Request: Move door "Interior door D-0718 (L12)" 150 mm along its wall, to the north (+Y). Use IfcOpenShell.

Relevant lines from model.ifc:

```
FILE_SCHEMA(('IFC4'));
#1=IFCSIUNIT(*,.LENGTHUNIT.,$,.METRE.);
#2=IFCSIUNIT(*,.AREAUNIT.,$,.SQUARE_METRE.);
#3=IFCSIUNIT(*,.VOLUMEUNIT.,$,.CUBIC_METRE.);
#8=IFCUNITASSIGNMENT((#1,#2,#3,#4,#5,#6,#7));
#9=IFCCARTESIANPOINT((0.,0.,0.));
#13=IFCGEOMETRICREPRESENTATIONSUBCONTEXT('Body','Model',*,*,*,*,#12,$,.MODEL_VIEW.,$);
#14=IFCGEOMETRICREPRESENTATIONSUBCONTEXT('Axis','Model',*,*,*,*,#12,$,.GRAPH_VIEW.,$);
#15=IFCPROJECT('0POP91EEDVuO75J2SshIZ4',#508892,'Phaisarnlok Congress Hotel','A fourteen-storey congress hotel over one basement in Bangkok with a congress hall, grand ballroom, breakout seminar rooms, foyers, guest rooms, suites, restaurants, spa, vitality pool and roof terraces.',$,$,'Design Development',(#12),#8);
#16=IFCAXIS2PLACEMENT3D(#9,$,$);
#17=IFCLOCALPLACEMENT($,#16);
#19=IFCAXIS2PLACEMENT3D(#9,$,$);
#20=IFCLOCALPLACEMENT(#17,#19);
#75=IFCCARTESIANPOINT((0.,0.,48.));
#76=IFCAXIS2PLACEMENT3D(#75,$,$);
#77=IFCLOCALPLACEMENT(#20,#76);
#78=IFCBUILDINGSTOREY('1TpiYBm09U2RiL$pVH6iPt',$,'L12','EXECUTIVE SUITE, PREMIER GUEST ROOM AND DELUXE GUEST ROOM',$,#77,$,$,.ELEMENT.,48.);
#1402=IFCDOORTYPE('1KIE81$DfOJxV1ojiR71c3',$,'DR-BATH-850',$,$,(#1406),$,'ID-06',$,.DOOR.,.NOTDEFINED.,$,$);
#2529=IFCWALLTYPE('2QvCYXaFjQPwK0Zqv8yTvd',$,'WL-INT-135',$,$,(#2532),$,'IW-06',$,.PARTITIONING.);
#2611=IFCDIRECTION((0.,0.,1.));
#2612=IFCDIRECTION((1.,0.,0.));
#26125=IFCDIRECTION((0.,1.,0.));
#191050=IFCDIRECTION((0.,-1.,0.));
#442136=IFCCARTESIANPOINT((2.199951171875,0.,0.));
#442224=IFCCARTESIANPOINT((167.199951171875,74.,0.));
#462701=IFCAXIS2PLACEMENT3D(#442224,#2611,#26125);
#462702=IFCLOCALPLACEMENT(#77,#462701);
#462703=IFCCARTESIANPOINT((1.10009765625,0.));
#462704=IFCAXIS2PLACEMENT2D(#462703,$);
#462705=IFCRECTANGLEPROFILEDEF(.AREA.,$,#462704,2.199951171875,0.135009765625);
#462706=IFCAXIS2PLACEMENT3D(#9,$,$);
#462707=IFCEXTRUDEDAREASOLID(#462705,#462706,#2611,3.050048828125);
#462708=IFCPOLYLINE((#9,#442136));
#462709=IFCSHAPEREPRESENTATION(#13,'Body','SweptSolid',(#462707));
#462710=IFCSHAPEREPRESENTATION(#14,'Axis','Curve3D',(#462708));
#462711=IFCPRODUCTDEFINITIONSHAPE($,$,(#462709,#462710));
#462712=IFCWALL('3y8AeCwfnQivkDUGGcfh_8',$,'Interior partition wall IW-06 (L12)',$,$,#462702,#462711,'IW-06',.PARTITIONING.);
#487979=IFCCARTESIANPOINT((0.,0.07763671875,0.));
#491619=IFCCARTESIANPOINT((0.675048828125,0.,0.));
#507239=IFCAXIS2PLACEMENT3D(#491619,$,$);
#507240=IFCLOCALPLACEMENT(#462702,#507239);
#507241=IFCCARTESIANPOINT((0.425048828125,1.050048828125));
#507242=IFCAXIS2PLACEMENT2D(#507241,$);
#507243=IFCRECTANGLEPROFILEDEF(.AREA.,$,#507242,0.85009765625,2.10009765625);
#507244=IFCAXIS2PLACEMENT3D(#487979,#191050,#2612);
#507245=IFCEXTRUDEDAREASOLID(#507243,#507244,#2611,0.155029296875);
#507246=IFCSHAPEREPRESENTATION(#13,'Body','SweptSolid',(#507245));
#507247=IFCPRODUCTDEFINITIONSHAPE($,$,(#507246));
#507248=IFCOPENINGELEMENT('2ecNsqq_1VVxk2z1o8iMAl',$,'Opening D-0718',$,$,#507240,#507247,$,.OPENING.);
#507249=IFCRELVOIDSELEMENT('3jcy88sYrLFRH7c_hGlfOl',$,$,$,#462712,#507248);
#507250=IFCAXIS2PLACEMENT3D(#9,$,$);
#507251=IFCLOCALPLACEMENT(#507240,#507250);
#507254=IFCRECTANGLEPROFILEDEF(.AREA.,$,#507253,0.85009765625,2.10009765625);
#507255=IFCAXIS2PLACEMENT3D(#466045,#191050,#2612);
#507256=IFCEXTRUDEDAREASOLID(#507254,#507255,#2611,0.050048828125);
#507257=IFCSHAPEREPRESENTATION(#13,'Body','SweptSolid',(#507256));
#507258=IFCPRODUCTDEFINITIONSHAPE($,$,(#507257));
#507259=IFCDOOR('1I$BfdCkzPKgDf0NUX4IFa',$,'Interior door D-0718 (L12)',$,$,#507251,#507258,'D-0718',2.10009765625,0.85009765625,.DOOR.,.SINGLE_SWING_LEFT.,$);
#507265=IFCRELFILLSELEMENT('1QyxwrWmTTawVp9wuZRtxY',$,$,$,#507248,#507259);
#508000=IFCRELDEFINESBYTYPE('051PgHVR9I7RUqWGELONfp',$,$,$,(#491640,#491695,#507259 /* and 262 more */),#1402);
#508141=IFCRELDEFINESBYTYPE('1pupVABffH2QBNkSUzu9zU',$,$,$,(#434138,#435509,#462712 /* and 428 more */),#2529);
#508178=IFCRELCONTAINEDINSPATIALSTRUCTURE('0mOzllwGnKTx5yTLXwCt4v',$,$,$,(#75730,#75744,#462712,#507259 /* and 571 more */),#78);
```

```python
import ifcopenshell
import ifcopenshell.api.geometry
import ifcopenshell.util.placement
import ifcopenshell.util.unit

model = ifcopenshell.open("model.ifc")
unit_scale = ifcopenshell.util.unit.calculate_unit_scale(model)

door = model.by_guid("1I$BfdCkzPKgDf0NUX4IFa")
opening = door.FillsVoids[0].RelatingOpeningElement
wall = opening.VoidsElements[0].RelatingBuildingElement

wall_matrix = ifcopenshell.util.placement.get_local_placement(wall.ObjectPlacement)
shift = wall_matrix[:3, 0] * 0.15 / unit_scale
before = ifcopenshell.util.placement.get_local_placement(door.ObjectPlacement)[:3, 3].copy()

# The door is placed relative to its opening, so it follows when the opening moves.
matrix = ifcopenshell.util.placement.get_local_placement(opening.ObjectPlacement)
matrix[:3, 3] += shift
ifcopenshell.api.geometry.edit_object_placement(
    model, product=opening, matrix=matrix, is_si=False, should_transform_children=True
)

after = ifcopenshell.util.placement.get_local_placement(door.ObjectPlacement)[:3, 3]
print("door moved by", (after - before).round(3) + 0.0)

model.write("model_rev.ifc")
```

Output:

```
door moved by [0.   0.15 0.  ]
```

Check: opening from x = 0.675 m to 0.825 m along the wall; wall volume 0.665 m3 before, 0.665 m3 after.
